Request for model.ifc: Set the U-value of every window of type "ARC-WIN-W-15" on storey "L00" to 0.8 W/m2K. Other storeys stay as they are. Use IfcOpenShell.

First a look at what the model holds.

```python
import ifcopenshell
import ifcopenshell.util.element

model = ifcopenshell.open("model.ifc")
print(model.schema)
storey = next(s for s in model.by_type("IfcBuildingStorey") if s.Name == "L00")
windows = [e for e in ifcopenshell.util.element.get_decomposition(storey) if e.is_a("IfcWindow")]
seen = {}
for e in windows:
    element_type = ifcopenshell.util.element.get_type(e)
    key = (element_type.Name if element_type != e and element_type else None, ifcopenshell.util.element.get_pset(e, "Pset_WindowCommon", "ThermalTransmittance"))
    seen[key] = seen.get(key, 0) + 1
for (name, value), count in sorted(seen.items(), key=str):
    print(count, "x", name, "|", value)
```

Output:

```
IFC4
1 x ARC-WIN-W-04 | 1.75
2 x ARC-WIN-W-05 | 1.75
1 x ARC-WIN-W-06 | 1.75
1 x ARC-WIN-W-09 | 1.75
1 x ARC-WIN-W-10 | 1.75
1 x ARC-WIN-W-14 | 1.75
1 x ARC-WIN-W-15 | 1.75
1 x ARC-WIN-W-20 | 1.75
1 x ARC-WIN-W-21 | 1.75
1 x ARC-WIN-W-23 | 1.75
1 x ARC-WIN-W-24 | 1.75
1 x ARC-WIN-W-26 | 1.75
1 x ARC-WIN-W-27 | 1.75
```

```python
import ifcopenshell
import ifcopenshell.api.pset
import ifcopenshell.util.element

model = ifcopenshell.open("model.ifc")

storey = next(s for s in model.by_type("IfcBuildingStorey") if s.Name == "L00")
windows = [e for e in ifcopenshell.util.element.get_decomposition(storey) if e.is_a("IfcWindow")]

count = 0
for e in windows:
    element_type = ifcopenshell.util.element.get_type(e)
    if element_type in (None, e) or element_type.Name != "ARC-WIN-W-15":
        continue
    # add_pset returns the element's existing set when there is one.
    pset = ifcopenshell.api.pset.add_pset(model, product=e, name="Pset_WindowCommon")
    ifcopenshell.api.pset.edit_pset(model, pset=pset, properties={"ThermalTransmittance": 0.8})
    count += 1

print(count, "windows updated")

model.write("model_rev.ifc")
```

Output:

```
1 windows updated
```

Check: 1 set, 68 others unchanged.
